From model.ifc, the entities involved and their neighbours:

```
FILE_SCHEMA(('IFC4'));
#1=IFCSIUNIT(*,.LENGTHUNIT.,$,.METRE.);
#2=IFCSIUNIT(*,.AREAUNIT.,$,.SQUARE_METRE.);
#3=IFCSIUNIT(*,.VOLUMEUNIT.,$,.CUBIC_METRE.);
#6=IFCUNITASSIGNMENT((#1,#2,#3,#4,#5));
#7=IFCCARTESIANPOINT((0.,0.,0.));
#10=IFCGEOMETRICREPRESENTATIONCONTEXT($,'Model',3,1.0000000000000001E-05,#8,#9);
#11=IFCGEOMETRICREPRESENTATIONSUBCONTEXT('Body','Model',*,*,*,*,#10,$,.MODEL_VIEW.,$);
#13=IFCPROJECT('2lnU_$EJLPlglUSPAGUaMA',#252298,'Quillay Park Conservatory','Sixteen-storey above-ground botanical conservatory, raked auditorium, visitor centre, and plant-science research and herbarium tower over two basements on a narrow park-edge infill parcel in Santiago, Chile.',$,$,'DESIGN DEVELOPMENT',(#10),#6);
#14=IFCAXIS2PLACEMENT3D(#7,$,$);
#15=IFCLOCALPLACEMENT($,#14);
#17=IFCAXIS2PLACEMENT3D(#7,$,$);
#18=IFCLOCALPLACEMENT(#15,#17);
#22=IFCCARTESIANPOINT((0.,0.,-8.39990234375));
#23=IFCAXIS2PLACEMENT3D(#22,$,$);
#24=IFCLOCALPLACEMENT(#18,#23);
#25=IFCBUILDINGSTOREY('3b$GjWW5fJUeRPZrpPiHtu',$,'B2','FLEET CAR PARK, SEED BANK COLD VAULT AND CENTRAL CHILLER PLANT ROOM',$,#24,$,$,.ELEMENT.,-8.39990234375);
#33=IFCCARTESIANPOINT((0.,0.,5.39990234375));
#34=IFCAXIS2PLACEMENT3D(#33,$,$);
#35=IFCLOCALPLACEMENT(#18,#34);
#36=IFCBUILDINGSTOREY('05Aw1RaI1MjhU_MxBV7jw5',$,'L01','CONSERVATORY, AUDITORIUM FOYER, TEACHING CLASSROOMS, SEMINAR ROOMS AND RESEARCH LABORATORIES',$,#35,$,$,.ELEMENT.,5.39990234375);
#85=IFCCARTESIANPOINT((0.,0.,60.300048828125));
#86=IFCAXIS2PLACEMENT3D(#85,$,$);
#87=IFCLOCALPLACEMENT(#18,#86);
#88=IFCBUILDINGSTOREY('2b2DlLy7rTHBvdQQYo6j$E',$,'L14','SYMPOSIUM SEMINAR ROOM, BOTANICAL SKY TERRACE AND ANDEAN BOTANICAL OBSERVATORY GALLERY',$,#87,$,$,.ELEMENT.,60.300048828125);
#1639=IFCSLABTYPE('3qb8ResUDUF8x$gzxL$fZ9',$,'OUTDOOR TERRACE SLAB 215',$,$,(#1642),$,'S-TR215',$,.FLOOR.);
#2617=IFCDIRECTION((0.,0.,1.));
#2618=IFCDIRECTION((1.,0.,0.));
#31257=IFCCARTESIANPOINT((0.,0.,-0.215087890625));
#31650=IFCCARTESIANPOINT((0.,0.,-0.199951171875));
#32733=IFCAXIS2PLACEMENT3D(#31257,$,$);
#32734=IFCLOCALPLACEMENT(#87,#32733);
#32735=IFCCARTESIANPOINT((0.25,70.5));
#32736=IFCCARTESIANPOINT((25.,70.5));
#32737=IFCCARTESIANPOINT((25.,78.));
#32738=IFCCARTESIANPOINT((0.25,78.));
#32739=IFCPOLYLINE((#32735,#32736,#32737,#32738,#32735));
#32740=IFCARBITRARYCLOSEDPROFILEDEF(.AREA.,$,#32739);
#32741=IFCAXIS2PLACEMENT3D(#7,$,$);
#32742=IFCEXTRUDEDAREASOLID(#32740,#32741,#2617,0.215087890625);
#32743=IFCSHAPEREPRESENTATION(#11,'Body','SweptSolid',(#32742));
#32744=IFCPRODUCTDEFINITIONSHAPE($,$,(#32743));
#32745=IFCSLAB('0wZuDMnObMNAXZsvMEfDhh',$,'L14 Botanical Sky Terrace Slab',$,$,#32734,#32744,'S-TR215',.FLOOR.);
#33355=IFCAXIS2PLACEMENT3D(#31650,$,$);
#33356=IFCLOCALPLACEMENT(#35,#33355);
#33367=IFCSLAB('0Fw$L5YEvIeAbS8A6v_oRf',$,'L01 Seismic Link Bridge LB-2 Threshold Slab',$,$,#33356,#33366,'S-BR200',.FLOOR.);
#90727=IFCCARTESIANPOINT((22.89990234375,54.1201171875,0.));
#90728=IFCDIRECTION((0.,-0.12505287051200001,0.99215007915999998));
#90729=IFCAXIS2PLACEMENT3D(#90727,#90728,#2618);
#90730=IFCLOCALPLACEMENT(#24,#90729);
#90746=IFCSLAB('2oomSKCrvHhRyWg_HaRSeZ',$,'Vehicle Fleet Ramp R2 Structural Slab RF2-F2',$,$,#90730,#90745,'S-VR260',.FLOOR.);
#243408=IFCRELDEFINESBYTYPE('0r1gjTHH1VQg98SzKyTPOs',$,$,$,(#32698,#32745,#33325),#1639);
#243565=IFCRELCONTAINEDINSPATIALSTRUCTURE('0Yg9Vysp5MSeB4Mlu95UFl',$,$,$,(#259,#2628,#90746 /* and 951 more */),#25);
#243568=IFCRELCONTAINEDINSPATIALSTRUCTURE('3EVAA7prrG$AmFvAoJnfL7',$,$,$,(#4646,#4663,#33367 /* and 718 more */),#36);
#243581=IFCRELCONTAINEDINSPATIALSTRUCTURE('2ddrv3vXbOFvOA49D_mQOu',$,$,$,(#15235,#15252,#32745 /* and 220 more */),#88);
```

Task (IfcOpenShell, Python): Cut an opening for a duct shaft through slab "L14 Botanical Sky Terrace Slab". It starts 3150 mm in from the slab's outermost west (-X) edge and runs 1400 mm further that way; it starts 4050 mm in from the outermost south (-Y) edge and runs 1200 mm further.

```python
import numpy as np
import ifcopenshell
import ifcopenshell.api.feature
import ifcopenshell.api.geometry
import ifcopenshell.api.root
import ifcopenshell.geom
import ifcopenshell.util.placement
import ifcopenshell.util.representation
import ifcopenshell.util.shape
import ifcopenshell.util.unit

model = ifcopenshell.open("model.ifc")
unit_scale = ifcopenshell.util.unit.calculate_unit_scale(model)
settings = ifcopenshell.geom.settings()


def volume(element):
    """Net volume in cubic metres, openings subtracted."""
    shape = ifcopenshell.geom.create_shape(settings, element)
    return ifcopenshell.util.shape.get_volume(shape.geometry)


slab = model.by_guid("0wZuDMnObMNAXZsvMEfDhh")
before = volume(slab)

# Extent in the slab's own axes, in metres. The edges named are its -X and -Y sides.
slab_shape = ifcopenshell.geom.create_shape(settings, slab)
vertices = ifcopenshell.util.shape.get_vertices(slab_shape.geometry)
x_min, y_min, bottom = vertices.min(axis=0)
top = vertices[:, 2].max()

opening = ifcopenshell.api.root.create_entity(model, ifc_class="IfcOpeningElement", name="Duct shaft opening", predefined_type="OPENING")
context = ifcopenshell.util.representation.get_context(model, "Model", "Body", "MODEL_VIEW")
width, depth = 1.4, 1.2
outline = [(0.0, 0.0), (width, 0.0), (width, depth), (0.0, depth), (0.0, 0.0)]
# Overshoot both faces by 50 mm so the cut is clean.
shape = ifcopenshell.api.geometry.add_slab_representation(
    model, context=context, depth=top - bottom + 0.1, polyline=outline
)
ifcopenshell.api.geometry.assign_representation(model, product=opening, representation=shape)

matrix = ifcopenshell.util.placement.get_local_placement(slab.ObjectPlacement)
matrix[:, 3] = matrix @ np.append(np.array([x_min + 3.15, y_min + 4.05, bottom - 0.05]) / unit_scale, 1.0)
ifcopenshell.api.geometry.edit_object_placement(model, product=opening, matrix=matrix, is_si=False)
ifcopenshell.api.feature.add_feature(model, feature=opening, element=slab)

after = volume(slab)

print(f"slab volume {before:.3f} -> {after:.3f} m3")

model.write("model_rev.ifc")
```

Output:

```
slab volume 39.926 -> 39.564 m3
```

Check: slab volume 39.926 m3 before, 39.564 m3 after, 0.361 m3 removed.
